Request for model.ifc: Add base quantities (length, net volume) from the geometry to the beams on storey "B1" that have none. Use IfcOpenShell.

First a look at what the model holds.

```python
import ifcopenshell
import ifcopenshell.util.element
import ifcopenshell.util.unit

model = ifcopenshell.open("model.ifc")
print(model.schema)
for unit_type in ("LENGTHUNIT", "AREAUNIT", "VOLUMEUNIT"):
    print(unit_type, ifcopenshell.util.unit.calculate_unit_scale(model, unit_type))
storey = next(s for s in model.by_type("IfcBuildingStorey") if s.Name == "B1")
beams = [e for e in ifcopenshell.util.element.get_decomposition(storey) if e.is_a("IfcBeam")]
for e in sorted(beams, key=lambda e: e.id()):
    print(e.id(), e.is_a(), e.Name, list(ifcopenshell.util.element.get_psets(e, qtos_only=True)), sep=" | ")
```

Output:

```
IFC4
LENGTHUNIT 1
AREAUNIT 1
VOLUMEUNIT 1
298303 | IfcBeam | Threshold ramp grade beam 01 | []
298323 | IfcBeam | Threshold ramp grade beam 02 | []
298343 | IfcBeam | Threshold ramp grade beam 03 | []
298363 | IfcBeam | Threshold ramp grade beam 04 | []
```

```python
import ifcopenshell
import ifcopenshell.api.pset
import ifcopenshell.geom
import ifcopenshell.util.element
import ifcopenshell.util.shape
import ifcopenshell.util.unit

model = ifcopenshell.open("model.ifc")
unit_scale = ifcopenshell.util.unit.calculate_unit_scale(model)
volume_scale = ifcopenshell.util.unit.calculate_unit_scale(model, "VOLUMEUNIT")
settings = ifcopenshell.geom.settings()

storey = next(s for s in model.by_type("IfcBuildingStorey") if s.Name == "B1")
beams = [e for e in ifcopenshell.util.element.get_decomposition(storey) if e.is_a("IfcBeam")]

for e in sorted(beams, key=lambda e: e.id()):
    if ifcopenshell.util.element.get_psets(e, qtos_only=True, should_inherit=False):
        continue
    # Geometry comes back in metres, in the element's own axes.
    shape = ifcopenshell.geom.create_shape(settings, e)
    values = {
        "Length": ifcopenshell.util.shape.get_max_xyz(shape.geometry) / unit_scale,
        "NetVolume": ifcopenshell.util.shape.get_volume(shape.geometry) / volume_scale,
    }
    qto = ifcopenshell.api.pset.add_qto(model, product=e, name="Qto_BeamBaseQuantities")
    ifcopenshell.api.pset.edit_qto(model, qto=qto, properties=values)
    print(e.id(), {k: round(v, 3) for k, v in values.items()})

model.write("model_v2.ifc")
```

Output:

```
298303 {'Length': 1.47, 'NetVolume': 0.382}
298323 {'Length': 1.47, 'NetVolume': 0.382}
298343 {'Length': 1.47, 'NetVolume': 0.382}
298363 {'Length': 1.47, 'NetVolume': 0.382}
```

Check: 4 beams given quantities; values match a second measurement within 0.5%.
